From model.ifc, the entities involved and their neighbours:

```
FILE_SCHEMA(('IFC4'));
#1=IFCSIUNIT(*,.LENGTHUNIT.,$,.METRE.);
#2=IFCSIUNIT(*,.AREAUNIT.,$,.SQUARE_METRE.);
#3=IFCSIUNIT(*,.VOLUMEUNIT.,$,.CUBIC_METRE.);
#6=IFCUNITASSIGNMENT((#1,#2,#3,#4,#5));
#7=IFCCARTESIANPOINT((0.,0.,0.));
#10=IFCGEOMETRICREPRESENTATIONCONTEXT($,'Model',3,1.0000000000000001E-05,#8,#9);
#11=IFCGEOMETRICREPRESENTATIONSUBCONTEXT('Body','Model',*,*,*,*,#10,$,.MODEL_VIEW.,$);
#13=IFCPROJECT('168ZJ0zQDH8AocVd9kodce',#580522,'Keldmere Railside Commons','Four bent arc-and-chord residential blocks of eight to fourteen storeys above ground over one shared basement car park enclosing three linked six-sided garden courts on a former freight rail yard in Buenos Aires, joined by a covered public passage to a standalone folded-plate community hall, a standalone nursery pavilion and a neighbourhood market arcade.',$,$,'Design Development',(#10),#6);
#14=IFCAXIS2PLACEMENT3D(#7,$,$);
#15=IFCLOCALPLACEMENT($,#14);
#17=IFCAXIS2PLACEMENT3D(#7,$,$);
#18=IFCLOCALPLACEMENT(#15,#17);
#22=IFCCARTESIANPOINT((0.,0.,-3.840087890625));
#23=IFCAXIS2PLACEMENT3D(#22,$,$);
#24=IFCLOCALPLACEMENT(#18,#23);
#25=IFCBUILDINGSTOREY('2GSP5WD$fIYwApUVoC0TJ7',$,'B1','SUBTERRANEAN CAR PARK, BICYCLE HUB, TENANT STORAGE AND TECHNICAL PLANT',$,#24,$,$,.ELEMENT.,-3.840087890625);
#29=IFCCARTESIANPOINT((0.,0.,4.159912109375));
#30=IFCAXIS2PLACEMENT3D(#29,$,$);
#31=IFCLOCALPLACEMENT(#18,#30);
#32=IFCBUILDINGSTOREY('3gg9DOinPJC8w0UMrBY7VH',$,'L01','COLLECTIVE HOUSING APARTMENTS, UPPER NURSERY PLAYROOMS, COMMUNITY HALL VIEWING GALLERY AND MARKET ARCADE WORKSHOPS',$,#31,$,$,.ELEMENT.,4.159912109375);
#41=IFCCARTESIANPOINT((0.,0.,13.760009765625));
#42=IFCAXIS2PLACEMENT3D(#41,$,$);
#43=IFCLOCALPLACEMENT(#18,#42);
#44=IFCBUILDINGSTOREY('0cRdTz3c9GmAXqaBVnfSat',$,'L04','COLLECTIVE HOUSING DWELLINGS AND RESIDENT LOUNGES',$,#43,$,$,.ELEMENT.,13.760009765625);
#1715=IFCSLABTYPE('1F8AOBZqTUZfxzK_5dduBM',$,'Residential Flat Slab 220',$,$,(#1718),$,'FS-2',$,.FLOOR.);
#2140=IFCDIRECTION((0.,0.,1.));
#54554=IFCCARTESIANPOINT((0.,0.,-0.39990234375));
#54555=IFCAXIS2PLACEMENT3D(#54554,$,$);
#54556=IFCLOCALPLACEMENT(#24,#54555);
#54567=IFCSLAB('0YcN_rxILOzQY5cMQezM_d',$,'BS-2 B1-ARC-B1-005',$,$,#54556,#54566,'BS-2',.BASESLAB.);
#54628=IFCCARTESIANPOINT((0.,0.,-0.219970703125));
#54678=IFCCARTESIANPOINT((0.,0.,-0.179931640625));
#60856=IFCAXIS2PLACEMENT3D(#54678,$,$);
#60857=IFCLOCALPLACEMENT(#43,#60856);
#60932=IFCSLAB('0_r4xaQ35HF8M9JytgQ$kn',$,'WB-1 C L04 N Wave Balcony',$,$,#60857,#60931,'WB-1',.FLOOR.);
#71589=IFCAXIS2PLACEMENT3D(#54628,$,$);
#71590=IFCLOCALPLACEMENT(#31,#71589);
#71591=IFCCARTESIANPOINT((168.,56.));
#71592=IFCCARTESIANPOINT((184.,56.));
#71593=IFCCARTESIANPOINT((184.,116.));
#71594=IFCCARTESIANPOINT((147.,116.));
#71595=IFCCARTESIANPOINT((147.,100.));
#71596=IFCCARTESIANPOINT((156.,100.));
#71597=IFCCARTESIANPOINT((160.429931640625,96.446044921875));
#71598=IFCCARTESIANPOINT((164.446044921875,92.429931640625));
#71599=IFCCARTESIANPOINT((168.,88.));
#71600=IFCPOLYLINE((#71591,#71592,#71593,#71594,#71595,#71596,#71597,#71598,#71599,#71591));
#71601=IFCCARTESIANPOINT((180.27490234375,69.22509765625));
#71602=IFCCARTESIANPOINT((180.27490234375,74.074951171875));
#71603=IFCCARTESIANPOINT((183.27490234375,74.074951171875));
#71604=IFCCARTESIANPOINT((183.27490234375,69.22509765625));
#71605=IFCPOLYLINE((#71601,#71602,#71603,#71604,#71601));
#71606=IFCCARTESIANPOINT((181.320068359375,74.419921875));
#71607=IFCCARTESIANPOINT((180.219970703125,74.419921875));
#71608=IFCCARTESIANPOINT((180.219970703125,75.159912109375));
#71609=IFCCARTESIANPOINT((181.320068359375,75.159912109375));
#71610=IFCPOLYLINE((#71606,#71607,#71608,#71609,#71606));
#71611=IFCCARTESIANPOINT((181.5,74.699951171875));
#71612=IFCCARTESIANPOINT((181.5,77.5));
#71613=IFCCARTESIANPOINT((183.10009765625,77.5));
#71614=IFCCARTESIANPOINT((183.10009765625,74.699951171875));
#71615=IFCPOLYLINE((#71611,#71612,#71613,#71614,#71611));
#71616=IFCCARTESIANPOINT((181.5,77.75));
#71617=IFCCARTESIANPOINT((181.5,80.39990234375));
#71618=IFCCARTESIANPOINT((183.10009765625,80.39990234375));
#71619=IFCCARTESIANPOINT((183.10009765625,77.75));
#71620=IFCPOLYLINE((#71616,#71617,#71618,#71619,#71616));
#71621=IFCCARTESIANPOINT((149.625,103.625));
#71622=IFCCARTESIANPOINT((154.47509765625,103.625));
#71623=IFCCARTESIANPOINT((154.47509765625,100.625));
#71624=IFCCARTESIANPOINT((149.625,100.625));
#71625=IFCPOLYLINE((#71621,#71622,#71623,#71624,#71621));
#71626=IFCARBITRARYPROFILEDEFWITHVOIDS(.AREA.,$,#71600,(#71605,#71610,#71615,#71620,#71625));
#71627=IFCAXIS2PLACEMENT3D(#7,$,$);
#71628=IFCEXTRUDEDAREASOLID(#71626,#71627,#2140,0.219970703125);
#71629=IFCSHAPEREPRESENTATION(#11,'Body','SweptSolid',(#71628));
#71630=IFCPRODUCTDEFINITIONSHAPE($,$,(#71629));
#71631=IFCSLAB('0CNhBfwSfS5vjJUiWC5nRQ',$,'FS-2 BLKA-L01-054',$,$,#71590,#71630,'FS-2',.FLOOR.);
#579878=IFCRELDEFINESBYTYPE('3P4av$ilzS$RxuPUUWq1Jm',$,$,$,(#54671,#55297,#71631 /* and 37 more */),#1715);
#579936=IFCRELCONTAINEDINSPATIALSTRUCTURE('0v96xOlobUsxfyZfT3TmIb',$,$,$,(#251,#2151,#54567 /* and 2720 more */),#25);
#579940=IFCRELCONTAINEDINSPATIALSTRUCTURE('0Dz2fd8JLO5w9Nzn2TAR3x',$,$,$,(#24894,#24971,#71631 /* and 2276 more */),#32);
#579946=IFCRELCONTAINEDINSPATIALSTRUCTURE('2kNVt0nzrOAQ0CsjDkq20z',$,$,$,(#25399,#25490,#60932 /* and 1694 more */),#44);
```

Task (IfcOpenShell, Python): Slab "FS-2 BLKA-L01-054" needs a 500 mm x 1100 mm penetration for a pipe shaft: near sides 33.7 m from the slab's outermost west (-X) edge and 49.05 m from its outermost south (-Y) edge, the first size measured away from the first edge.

```python
import numpy as np
import ifcopenshell
import ifcopenshell.api.feature
import ifcopenshell.api.geometry
import ifcopenshell.api.root
import ifcopenshell.geom
import ifcopenshell.util.placement
import ifcopenshell.util.representation
import ifcopenshell.util.shape
import ifcopenshell.util.unit

model = ifcopenshell.open("model.ifc")
unit_scale = ifcopenshell.util.unit.calculate_unit_scale(model)
settings = ifcopenshell.geom.settings()


def volume(element):
    """Net volume in cubic metres, openings subtracted."""
    shape = ifcopenshell.geom.create_shape(settings, element)
    return ifcopenshell.util.shape.get_volume(shape.geometry)


slab = model.by_guid("0CNhBfwSfS5vjJUiWC5nRQ")
before = volume(slab)

# Extent in the slab's own axes, in metres. The edges named are its -X and -Y sides.
slab_shape = ifcopenshell.geom.create_shape(settings, slab)
vertices = ifcopenshell.util.shape.get_vertices(slab_shape.geometry)
x_min, y_min, bottom = vertices.min(axis=0)
top = vertices[:, 2].max()

opening = ifcopenshell.api.root.create_entity(model, ifc_class="IfcOpeningElement", name="Pipe shaft opening", predefined_type="OPENING")
context = ifcopenshell.util.representation.get_context(model, "Model", "Body", "MODEL_VIEW")
width, depth = 0.5, 1.1
outline = [(0.0, 0.0), (width, 0.0), (width, depth), (0.0, depth), (0.0, 0.0)]
# Overshoot both faces by 50 mm so the cut is clean.
shape = ifcopenshell.api.geometry.add_slab_representation(
    model, context=context, depth=top - bottom + 0.1, polyline=outline
)
ifcopenshell.api.geometry.assign_representation(model, product=opening, representation=shape)

matrix = ifcopenshell.util.placement.get_local_placement(slab.ObjectPlacement)
matrix[:, 3] = matrix @ np.append(np.array([x_min + 33.7, y_min + 49.05, bottom - 0.05]) / unit_scale, 1.0)
ifcopenshell.api.geometry.edit_object_placement(model, product=opening, matrix=matrix, is_si=False)
ifcopenshell.api.feature.add_feature(model, feature=opening, element=slab)

after = volume(slab)

print(f"slab volume {before:.3f} -> {after:.3f} m3")

model.write("model_rev.ifc")
```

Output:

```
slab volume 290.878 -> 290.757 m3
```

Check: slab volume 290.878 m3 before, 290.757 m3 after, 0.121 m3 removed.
